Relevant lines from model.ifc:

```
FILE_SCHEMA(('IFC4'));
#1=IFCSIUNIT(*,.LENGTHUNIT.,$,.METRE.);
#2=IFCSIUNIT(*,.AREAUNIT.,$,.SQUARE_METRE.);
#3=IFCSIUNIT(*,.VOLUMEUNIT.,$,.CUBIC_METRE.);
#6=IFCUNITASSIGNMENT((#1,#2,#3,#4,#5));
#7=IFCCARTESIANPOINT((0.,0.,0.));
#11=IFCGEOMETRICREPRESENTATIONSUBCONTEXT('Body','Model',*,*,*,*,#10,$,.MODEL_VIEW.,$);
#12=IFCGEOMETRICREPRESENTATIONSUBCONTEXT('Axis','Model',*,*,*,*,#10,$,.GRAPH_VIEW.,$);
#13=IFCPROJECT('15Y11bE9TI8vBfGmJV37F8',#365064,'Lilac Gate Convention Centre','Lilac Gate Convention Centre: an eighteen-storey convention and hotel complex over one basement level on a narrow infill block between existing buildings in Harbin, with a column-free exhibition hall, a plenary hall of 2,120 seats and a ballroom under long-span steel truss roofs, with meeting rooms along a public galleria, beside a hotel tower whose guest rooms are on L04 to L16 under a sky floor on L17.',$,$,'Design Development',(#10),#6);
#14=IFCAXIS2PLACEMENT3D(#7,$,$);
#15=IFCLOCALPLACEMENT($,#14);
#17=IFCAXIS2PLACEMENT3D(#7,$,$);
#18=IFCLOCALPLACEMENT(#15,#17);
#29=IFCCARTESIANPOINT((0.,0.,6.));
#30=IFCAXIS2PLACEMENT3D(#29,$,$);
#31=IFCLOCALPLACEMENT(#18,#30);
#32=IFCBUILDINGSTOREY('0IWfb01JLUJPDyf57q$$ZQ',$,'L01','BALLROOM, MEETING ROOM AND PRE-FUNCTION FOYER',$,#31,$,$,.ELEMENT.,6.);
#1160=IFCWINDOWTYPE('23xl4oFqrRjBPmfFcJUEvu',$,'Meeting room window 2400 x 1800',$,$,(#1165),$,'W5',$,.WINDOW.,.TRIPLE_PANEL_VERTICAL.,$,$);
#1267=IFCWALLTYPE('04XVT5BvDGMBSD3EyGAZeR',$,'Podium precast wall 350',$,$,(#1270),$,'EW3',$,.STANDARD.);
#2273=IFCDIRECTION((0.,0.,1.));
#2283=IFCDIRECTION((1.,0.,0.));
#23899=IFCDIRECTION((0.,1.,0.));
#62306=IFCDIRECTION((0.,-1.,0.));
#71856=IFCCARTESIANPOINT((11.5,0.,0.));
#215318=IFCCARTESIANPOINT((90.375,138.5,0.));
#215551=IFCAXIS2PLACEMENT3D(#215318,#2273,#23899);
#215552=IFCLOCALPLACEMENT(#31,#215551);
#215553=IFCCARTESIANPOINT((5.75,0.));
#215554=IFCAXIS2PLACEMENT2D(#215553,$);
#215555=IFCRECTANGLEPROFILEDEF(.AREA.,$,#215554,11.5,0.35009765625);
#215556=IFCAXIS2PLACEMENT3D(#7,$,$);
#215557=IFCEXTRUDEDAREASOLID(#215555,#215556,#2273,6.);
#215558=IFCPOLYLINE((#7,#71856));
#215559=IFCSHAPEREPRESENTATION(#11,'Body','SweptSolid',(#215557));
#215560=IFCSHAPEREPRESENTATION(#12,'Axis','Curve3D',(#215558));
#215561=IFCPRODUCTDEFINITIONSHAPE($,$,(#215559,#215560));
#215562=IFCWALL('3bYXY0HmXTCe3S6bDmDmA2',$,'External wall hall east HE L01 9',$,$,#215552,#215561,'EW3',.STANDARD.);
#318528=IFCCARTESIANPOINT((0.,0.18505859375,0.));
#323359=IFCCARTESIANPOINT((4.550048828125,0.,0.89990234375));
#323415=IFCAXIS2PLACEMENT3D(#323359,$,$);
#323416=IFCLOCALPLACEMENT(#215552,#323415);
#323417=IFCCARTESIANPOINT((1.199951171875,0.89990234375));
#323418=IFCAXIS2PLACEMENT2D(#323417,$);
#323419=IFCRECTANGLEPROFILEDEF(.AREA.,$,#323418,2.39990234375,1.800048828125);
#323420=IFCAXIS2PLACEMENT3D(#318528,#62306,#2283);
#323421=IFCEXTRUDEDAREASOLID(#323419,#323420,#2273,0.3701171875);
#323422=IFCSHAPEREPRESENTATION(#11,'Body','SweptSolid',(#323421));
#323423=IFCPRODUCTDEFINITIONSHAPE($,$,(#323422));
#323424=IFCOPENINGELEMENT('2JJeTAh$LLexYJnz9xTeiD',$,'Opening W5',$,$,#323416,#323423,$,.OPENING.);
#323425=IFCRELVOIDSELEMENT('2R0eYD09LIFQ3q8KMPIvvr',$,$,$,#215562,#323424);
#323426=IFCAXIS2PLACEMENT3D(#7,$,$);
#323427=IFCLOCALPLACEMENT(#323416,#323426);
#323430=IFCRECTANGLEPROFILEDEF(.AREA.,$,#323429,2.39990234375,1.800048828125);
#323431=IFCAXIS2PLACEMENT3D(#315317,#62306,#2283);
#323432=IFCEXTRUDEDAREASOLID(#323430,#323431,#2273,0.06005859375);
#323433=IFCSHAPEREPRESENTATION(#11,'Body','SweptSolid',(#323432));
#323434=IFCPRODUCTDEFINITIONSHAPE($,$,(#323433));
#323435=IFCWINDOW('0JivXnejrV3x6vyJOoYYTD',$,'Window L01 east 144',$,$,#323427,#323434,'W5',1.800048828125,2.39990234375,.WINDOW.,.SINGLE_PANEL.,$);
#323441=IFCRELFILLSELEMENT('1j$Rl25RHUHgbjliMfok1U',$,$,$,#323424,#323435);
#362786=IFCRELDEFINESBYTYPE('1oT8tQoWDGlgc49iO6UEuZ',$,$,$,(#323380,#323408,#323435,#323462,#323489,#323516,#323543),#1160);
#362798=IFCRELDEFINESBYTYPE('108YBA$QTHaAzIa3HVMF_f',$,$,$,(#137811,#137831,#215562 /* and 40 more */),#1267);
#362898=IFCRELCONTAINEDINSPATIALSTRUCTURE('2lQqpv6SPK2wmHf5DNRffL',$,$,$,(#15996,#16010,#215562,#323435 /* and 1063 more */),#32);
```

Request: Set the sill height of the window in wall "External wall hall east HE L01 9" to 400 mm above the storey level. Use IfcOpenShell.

```python
import numpy as np
import ifcopenshell
import ifcopenshell.api.geometry
import ifcopenshell.geom
import ifcopenshell.util.element
import ifcopenshell.util.placement
import ifcopenshell.util.shape
import ifcopenshell.util.unit

model = ifcopenshell.open("model.ifc")
unit_scale = ifcopenshell.util.unit.calculate_unit_scale(model)

window = model.by_guid("0JivXnejrV3x6vyJOoYYTD")
opening = window.FillsVoids[0].RelatingOpeningElement
storey = ifcopenshell.util.element.get_container(window, ifc_class="IfcBuildingStorey")
level = ifcopenshell.util.placement.get_local_placement(storey.ObjectPlacement)[2, 3]

# The opening's origin need not be at the sill, so measure its lowest point.
shape = ifcopenshell.geom.create_shape(ifcopenshell.geom.settings(), opening)
bottom = ifcopenshell.util.shape.get_shape_bottom_elevation(shape, shape.geometry) / unit_scale
dz = level + 0.4 / unit_scale - bottom

shift = np.array([0.0, 0.0, dz])
# The window is placed relative to its opening, so it follows when the opening moves.
matrix = ifcopenshell.util.placement.get_local_placement(opening.ObjectPlacement)
matrix[:3, 3] += shift
ifcopenshell.api.geometry.edit_object_placement(
    model, product=opening, matrix=matrix, is_si=False, should_transform_children=True
)

print(f"moved by {dz * unit_scale:+.3f} m")

model.write("model-out.ifc")
```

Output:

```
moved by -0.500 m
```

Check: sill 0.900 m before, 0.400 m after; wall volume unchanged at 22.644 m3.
